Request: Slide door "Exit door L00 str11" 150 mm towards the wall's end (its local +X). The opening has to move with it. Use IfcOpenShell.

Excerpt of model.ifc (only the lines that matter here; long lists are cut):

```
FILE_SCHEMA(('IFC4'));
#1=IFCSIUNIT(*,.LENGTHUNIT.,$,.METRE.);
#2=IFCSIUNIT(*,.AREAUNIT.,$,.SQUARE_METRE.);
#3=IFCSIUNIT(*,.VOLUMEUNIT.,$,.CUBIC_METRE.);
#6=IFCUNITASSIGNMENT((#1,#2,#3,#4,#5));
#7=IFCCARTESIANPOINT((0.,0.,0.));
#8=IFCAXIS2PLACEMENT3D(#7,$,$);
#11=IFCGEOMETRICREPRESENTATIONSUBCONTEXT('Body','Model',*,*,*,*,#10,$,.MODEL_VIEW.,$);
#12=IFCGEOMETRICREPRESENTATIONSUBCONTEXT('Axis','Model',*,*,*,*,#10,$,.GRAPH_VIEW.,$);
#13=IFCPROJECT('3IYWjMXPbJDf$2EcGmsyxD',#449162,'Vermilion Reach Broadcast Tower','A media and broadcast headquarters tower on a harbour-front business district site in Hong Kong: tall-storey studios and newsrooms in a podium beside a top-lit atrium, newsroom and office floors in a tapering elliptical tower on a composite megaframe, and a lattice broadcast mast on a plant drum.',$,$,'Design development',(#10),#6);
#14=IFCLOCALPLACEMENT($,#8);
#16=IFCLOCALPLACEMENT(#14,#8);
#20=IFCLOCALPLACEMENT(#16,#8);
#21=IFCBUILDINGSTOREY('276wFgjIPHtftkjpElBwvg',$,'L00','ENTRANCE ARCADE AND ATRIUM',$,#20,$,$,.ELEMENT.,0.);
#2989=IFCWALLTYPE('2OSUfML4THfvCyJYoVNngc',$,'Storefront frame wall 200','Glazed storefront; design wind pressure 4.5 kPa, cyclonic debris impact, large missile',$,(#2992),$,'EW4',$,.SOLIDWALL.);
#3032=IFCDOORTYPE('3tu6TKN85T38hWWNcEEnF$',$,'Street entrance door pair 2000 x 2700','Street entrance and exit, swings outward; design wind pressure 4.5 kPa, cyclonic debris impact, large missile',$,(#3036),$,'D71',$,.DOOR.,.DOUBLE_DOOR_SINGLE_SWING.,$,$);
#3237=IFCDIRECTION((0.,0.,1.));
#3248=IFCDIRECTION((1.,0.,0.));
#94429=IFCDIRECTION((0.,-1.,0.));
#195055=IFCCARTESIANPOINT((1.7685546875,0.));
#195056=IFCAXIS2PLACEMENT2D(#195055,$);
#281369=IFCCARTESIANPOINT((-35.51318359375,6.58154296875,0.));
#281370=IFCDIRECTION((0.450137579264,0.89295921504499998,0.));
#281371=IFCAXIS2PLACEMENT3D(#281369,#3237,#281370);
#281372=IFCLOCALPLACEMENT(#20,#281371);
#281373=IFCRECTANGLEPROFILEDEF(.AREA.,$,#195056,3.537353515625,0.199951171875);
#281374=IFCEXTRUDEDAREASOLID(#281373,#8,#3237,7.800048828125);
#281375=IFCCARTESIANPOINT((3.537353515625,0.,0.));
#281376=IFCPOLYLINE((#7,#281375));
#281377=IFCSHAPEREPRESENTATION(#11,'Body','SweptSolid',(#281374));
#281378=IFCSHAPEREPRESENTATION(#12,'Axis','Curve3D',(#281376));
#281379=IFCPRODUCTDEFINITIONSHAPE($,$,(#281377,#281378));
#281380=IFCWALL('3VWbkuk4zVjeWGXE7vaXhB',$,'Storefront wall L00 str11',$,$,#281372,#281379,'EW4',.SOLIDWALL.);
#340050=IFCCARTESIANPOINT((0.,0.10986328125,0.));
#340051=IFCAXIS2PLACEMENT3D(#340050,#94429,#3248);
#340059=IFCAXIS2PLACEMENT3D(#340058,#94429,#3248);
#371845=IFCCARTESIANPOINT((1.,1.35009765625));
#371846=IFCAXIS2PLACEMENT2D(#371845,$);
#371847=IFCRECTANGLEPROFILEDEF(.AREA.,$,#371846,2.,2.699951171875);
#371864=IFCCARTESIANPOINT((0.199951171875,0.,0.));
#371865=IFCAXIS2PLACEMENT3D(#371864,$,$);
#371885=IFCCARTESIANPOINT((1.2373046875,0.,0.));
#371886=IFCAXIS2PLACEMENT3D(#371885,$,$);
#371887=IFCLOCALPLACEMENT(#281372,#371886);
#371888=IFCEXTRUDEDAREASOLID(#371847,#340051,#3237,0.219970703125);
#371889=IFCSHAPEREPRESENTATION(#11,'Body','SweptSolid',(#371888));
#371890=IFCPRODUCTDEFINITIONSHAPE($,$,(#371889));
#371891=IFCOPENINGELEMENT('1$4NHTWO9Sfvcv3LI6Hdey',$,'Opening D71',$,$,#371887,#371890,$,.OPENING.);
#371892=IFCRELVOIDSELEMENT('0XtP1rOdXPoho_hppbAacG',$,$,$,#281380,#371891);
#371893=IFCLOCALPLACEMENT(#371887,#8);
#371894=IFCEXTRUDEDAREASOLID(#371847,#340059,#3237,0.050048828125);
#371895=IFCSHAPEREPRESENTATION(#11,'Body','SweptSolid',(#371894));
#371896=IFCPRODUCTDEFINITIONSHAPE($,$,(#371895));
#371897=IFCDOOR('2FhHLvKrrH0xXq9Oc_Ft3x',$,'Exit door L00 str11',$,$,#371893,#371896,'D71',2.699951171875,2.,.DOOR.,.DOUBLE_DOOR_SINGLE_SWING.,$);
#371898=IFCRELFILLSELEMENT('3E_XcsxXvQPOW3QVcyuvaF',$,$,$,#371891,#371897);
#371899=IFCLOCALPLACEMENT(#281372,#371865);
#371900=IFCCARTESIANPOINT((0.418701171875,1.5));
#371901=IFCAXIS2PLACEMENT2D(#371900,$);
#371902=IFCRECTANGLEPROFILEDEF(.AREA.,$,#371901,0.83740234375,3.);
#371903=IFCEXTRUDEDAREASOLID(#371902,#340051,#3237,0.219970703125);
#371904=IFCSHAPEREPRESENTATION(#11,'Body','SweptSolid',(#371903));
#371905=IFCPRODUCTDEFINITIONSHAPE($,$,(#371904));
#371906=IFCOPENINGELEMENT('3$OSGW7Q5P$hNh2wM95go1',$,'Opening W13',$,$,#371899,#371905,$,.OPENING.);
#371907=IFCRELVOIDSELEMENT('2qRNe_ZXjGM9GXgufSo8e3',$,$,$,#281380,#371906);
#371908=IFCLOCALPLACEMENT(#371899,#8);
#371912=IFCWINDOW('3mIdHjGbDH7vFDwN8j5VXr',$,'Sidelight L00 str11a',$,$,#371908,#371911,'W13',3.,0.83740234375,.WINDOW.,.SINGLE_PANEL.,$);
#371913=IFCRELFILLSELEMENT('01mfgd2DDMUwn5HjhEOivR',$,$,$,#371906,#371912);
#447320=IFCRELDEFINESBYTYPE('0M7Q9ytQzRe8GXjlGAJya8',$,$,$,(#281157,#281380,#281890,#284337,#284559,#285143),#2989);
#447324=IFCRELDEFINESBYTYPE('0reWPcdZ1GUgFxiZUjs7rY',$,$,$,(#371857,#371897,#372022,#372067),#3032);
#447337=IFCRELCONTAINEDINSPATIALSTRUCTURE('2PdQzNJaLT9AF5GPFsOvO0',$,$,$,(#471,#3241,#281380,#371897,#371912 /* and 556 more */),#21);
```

```python
import ifcopenshell
import ifcopenshell.api.geometry
import ifcopenshell.util.placement
import ifcopenshell.util.unit

model = ifcopenshell.open("model.ifc")
unit_scale = ifcopenshell.util.unit.calculate_unit_scale(model)

door = model.by_guid("2FhHLvKrrH0xXq9Oc_Ft3x")
opening = door.FillsVoids[0].RelatingOpeningElement
wall = opening.VoidsElements[0].RelatingBuildingElement

wall_matrix = ifcopenshell.util.placement.get_local_placement(wall.ObjectPlacement)
shift = wall_matrix[:3, 0] * 0.15 / unit_scale
before = ifcopenshell.util.placement.get_local_placement(door.ObjectPlacement)[:3, 3].copy()

# The door is placed relative to its opening, so it follows when the opening moves.
matrix = ifcopenshell.util.placement.get_local_placement(opening.ObjectPlacement)
matrix[:3, 3] += shift
ifcopenshell.api.geometry.edit_object_placement(
    model, product=opening, matrix=matrix, is_si=False, should_transform_children=True
)

after = ifcopenshell.util.placement.get_local_placement(door.ObjectPlacement)[:3, 3]
print("door moved by", (after - before).round(3) + 0.0)

model.write("model_rev.ifc")
```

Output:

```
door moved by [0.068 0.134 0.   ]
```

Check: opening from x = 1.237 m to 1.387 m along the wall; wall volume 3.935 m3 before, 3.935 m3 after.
